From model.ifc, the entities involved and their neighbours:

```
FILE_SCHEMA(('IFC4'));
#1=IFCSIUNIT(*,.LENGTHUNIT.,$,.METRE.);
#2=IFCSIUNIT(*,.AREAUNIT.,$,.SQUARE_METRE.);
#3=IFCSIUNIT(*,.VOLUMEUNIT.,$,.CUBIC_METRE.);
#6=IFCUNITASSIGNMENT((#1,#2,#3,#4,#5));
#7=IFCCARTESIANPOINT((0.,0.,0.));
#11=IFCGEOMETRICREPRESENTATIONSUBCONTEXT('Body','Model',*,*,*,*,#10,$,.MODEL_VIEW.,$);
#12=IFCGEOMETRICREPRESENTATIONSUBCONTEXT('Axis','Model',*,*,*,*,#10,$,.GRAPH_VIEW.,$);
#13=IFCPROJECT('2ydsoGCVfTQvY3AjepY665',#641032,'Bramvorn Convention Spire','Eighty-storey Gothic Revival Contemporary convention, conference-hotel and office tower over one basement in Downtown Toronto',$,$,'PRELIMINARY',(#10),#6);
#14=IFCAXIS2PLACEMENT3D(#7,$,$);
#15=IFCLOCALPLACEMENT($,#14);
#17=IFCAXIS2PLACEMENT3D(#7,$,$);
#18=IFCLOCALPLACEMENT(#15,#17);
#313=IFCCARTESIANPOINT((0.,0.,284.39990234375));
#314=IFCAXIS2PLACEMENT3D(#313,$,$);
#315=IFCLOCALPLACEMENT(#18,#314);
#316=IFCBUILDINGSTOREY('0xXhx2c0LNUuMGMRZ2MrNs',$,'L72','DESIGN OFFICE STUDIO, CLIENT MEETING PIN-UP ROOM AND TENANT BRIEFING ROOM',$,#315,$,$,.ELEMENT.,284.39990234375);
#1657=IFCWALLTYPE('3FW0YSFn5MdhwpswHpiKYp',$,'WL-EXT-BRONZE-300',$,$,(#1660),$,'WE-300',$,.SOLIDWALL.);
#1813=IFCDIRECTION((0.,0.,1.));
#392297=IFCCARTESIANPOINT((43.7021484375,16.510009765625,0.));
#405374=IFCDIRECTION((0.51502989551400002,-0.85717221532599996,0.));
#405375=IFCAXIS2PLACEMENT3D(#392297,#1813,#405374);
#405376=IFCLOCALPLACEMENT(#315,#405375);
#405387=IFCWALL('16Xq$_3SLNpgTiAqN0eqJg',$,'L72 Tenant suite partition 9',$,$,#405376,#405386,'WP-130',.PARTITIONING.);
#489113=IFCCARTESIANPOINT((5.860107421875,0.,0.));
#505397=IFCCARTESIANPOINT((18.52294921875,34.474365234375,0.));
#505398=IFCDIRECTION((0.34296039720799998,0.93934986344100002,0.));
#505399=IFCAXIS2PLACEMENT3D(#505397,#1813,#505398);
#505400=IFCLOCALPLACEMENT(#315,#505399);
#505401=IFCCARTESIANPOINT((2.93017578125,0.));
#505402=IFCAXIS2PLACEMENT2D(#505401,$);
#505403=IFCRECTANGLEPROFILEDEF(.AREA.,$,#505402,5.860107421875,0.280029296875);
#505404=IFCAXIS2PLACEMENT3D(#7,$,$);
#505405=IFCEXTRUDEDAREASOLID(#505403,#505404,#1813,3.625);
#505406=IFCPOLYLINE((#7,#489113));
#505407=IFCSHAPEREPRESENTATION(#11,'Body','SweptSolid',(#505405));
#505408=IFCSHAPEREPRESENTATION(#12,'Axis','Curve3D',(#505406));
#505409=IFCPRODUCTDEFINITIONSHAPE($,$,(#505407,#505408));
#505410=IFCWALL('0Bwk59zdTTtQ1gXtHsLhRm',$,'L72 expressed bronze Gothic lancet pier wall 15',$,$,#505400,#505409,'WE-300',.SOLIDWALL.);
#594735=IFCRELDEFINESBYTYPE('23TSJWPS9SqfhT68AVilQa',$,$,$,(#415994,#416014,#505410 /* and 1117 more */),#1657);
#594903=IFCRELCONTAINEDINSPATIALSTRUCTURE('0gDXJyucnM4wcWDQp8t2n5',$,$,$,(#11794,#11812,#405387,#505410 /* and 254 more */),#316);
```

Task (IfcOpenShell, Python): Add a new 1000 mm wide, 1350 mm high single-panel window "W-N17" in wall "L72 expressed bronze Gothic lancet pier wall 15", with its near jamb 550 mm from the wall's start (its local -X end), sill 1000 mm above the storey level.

```python
import numpy as np
import ifcopenshell
import ifcopenshell.api.feature
import ifcopenshell.api.geometry
import ifcopenshell.api.root
import ifcopenshell.api.spatial
import ifcopenshell.geom
import ifcopenshell.util.element
import ifcopenshell.util.placement
import ifcopenshell.util.representation
import ifcopenshell.util.shape
import ifcopenshell.util.unit

model = ifcopenshell.open("model.ifc")
unit_scale = ifcopenshell.util.unit.calculate_unit_scale(model)
settings = ifcopenshell.geom.settings()


def volume(element):
    """Net volume in cubic metres, openings subtracted."""
    shape = ifcopenshell.geom.create_shape(settings, element)
    return ifcopenshell.util.shape.get_volume(shape.geometry)


wall = model.by_id(505410)
storey = ifcopenshell.util.element.get_container(wall, ifc_class="IfcBuildingStorey")
context = ifcopenshell.util.representation.get_context(model, "Model", "Body", "MODEL_VIEW")
before = volume(wall)

width, height, from_end, sill = 1, 1.35, 0.55, 1  # metres

# The wall runs along its own X axis, and the end named is its -X end.
wall_shape = ifcopenshell.geom.create_shape(settings, wall)
x, y, z = ifcopenshell.util.shape.get_vertices(wall_shape.geometry).T
start = x.min() + from_end
face, thickness = float(y.min()), float(y.max() - y.min())
wall_matrix = ifcopenshell.util.placement.get_local_placement(wall.ObjectPlacement)
level = ifcopenshell.util.placement.get_local_placement(storey.ObjectPlacement)[2, 3]


def in_wall(x, y):
    """Placement at x, y metres in the wall's axes, at sill height."""
    matrix = wall_matrix.copy()
    matrix[:, 3] = wall_matrix @ np.array([x / unit_scale, y / unit_scale, 0.0, 1.0])
    matrix[2, 3] = level + sill / unit_scale
    return matrix


# Opening: a box that overshoots both wall faces by 50 mm.
opening = ifcopenshell.api.root.create_entity(model, ifc_class="IfcOpeningElement", predefined_type="OPENING")
box = ifcopenshell.api.geometry.add_wall_representation(
    model, context=context, length=width, height=height, thickness=thickness + 0.1
)
ifcopenshell.api.geometry.assign_representation(model, product=opening, representation=box)
ifcopenshell.api.geometry.edit_object_placement(model, product=opening, matrix=in_wall(start, face - 0.05), is_si=False)
ifcopenshell.api.feature.add_feature(model, feature=opening, element=wall)

window = ifcopenshell.api.root.create_entity(model, ifc_class="IfcWindow", name="W-N17", predefined_type="WINDOW")
window.OverallWidth, window.OverallHeight = width / unit_scale, height / unit_scale
window.PartitioningType = "SINGLE_PANEL"
body = ifcopenshell.api.geometry.add_window_representation(
    model,
    context=context,
    overall_width=window.OverallWidth,
    overall_height=window.OverallHeight,
    partition_type="SINGLE_PANEL",
)
ifcopenshell.api.geometry.assign_representation(model, product=window, representation=body)
ifcopenshell.api.spatial.assign_container(model, products=[window], relating_structure=storey)
ifcopenshell.api.feature.add_filling(model, opening=opening, element=window)

# Centre the window in the wall's thickness.
ifcopenshell.api.geometry.edit_object_placement(model, product=window, matrix=in_wall(start, face), is_si=False)
window_shape = ifcopenshell.geom.create_shape(settings, window)
depth = ifcopenshell.util.shape.get_vertices(window_shape.geometry)[:, 1]
offset = face + thickness / 2 - (depth.min() + depth.max()) / 2
ifcopenshell.api.geometry.edit_object_placement(model, product=window, matrix=in_wall(start, offset), is_si=False)

after = volume(wall)

print(f"wall volume {before:.3f} -> {after:.3f} m3")

model.write("model_v2.ifc")
```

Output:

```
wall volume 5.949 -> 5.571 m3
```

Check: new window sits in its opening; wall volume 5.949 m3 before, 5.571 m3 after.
